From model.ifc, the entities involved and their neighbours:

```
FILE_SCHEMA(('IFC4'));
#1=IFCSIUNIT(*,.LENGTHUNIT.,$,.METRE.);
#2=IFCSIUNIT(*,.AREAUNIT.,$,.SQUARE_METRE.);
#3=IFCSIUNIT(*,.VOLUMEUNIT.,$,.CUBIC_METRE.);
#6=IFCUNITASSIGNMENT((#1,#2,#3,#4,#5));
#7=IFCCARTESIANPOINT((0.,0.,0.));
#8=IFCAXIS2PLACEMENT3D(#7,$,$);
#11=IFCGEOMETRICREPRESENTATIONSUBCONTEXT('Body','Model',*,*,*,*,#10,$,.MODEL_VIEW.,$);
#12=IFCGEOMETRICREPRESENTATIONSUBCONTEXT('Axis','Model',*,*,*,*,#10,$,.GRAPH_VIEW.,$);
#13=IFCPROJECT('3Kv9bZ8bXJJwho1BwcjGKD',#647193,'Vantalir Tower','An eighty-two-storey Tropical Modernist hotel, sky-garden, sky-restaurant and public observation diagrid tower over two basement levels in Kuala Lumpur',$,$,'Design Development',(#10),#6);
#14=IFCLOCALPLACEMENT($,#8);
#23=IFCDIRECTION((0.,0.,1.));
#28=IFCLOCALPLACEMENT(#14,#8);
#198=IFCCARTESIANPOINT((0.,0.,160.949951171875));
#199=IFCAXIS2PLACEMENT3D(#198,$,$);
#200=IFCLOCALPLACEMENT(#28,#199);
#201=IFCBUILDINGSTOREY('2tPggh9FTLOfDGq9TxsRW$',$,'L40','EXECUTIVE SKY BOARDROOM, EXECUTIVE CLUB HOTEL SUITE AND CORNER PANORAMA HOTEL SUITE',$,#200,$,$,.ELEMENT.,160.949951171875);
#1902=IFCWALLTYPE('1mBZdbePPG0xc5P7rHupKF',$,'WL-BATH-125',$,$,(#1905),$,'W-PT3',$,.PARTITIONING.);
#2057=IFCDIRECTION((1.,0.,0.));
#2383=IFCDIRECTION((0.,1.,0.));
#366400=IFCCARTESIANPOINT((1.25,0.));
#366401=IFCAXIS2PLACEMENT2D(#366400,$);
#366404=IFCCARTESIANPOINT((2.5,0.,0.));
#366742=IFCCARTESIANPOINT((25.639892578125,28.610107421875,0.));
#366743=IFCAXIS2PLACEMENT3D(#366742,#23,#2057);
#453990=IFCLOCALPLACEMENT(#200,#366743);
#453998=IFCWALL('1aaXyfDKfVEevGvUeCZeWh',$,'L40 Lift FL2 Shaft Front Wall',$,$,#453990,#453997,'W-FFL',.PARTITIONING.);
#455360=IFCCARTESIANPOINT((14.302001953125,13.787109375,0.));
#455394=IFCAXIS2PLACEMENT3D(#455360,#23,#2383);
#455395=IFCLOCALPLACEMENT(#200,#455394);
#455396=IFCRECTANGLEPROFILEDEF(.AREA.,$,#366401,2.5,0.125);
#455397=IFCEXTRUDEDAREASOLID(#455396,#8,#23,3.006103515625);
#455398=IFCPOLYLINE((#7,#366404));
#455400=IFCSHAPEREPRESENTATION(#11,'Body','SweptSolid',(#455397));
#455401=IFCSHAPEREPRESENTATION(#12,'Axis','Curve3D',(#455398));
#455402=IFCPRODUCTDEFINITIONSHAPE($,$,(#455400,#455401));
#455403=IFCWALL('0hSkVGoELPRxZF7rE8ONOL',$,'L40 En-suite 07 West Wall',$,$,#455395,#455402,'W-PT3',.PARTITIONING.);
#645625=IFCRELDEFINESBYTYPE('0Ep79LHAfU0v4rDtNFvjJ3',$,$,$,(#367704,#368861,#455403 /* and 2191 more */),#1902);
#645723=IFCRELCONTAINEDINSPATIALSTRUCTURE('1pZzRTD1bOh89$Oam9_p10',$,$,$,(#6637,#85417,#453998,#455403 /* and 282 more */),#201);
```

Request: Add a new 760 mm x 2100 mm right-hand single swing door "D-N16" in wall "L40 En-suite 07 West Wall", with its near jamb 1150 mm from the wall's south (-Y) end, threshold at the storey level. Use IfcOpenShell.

```python
import numpy as np
import ifcopenshell
import ifcopenshell.api.feature
import ifcopenshell.api.geometry
import ifcopenshell.api.root
import ifcopenshell.api.spatial
import ifcopenshell.geom
import ifcopenshell.util.element
import ifcopenshell.util.placement
import ifcopenshell.util.representation
import ifcopenshell.util.shape
import ifcopenshell.util.unit

model = ifcopenshell.open("model.ifc")
unit_scale = ifcopenshell.util.unit.calculate_unit_scale(model)
settings = ifcopenshell.geom.settings()


def volume(element):
    """Net volume in cubic metres, openings subtracted."""
    shape = ifcopenshell.geom.create_shape(settings, element)
    return ifcopenshell.util.shape.get_volume(shape.geometry)


wall = model.by_guid("0hSkVGoELPRxZF7rE8ONOL")
storey = ifcopenshell.util.element.get_container(wall, ifc_class="IfcBuildingStorey")
context = ifcopenshell.util.representation.get_context(model, "Model", "Body", "MODEL_VIEW")
before = volume(wall)

width, height, from_end, sill = 0.76, 2.1, 1.15, 0.0  # metres

# The wall runs along its own X axis, and the end named is its -X end.
wall_shape = ifcopenshell.geom.create_shape(settings, wall)
x, y, z = ifcopenshell.util.shape.get_vertices(wall_shape.geometry).T
start = x.min() + from_end
face, thickness = float(y.min()), float(y.max() - y.min())
wall_matrix = ifcopenshell.util.placement.get_local_placement(wall.ObjectPlacement)
level = ifcopenshell.util.placement.get_local_placement(storey.ObjectPlacement)[2, 3]


def in_wall(x, y):
    """Placement at x, y metres in the wall's axes, at sill height."""
    matrix = wall_matrix.copy()
    matrix[:, 3] = wall_matrix @ np.array([x / unit_scale, y / unit_scale, 0.0, 1.0])
    matrix[2, 3] = level + sill / unit_scale
    return matrix


# Opening: a box that overshoots both wall faces by 50 mm.
opening = ifcopenshell.api.root.create_entity(model, ifc_class="IfcOpeningElement", predefined_type="OPENING")
box = ifcopenshell.api.geometry.add_wall_representation(
    model, context=context, length=width, height=height, thickness=thickness + 0.1
)
ifcopenshell.api.geometry.assign_representation(model, product=opening, representation=box)
ifcopenshell.api.geometry.edit_object_placement(model, product=opening, matrix=in_wall(start, face - 0.05), is_si=False)
ifcopenshell.api.feature.add_feature(model, feature=opening, element=wall)

door = ifcopenshell.api.root.create_entity(model, ifc_class="IfcDoor", name="D-N16", predefined_type="DOOR")
door.OverallWidth, door.OverallHeight = width / unit_scale, height / unit_scale
door.OperationType = "SINGLE_SWING_RIGHT"
body = ifcopenshell.api.geometry.add_door_representation(
    model,
    context=context,
    overall_width=door.OverallWidth,
    overall_height=door.OverallHeight,
    operation_type="SINGLE_SWING_RIGHT",
    lining_properties={"LiningDepth": thickness / unit_scale, "ThresholdDepth": thickness / unit_scale},
)
ifcopenshell.api.geometry.assign_representation(model, product=door, representation=body)
ifcopenshell.api.spatial.assign_container(model, products=[door], relating_structure=storey)
ifcopenshell.api.feature.add_filling(model, opening=opening, element=door)

# The lining spans the wall, so the door starts at the wall face.
ifcopenshell.api.geometry.edit_object_placement(model, product=door, matrix=in_wall(start, face), is_si=False)

after = volume(wall)

print(f"wall volume {before:.3f} -> {after:.3f} m3")

model.write("model_rev.ifc")
```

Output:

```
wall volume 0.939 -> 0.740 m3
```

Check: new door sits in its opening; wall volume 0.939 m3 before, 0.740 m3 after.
